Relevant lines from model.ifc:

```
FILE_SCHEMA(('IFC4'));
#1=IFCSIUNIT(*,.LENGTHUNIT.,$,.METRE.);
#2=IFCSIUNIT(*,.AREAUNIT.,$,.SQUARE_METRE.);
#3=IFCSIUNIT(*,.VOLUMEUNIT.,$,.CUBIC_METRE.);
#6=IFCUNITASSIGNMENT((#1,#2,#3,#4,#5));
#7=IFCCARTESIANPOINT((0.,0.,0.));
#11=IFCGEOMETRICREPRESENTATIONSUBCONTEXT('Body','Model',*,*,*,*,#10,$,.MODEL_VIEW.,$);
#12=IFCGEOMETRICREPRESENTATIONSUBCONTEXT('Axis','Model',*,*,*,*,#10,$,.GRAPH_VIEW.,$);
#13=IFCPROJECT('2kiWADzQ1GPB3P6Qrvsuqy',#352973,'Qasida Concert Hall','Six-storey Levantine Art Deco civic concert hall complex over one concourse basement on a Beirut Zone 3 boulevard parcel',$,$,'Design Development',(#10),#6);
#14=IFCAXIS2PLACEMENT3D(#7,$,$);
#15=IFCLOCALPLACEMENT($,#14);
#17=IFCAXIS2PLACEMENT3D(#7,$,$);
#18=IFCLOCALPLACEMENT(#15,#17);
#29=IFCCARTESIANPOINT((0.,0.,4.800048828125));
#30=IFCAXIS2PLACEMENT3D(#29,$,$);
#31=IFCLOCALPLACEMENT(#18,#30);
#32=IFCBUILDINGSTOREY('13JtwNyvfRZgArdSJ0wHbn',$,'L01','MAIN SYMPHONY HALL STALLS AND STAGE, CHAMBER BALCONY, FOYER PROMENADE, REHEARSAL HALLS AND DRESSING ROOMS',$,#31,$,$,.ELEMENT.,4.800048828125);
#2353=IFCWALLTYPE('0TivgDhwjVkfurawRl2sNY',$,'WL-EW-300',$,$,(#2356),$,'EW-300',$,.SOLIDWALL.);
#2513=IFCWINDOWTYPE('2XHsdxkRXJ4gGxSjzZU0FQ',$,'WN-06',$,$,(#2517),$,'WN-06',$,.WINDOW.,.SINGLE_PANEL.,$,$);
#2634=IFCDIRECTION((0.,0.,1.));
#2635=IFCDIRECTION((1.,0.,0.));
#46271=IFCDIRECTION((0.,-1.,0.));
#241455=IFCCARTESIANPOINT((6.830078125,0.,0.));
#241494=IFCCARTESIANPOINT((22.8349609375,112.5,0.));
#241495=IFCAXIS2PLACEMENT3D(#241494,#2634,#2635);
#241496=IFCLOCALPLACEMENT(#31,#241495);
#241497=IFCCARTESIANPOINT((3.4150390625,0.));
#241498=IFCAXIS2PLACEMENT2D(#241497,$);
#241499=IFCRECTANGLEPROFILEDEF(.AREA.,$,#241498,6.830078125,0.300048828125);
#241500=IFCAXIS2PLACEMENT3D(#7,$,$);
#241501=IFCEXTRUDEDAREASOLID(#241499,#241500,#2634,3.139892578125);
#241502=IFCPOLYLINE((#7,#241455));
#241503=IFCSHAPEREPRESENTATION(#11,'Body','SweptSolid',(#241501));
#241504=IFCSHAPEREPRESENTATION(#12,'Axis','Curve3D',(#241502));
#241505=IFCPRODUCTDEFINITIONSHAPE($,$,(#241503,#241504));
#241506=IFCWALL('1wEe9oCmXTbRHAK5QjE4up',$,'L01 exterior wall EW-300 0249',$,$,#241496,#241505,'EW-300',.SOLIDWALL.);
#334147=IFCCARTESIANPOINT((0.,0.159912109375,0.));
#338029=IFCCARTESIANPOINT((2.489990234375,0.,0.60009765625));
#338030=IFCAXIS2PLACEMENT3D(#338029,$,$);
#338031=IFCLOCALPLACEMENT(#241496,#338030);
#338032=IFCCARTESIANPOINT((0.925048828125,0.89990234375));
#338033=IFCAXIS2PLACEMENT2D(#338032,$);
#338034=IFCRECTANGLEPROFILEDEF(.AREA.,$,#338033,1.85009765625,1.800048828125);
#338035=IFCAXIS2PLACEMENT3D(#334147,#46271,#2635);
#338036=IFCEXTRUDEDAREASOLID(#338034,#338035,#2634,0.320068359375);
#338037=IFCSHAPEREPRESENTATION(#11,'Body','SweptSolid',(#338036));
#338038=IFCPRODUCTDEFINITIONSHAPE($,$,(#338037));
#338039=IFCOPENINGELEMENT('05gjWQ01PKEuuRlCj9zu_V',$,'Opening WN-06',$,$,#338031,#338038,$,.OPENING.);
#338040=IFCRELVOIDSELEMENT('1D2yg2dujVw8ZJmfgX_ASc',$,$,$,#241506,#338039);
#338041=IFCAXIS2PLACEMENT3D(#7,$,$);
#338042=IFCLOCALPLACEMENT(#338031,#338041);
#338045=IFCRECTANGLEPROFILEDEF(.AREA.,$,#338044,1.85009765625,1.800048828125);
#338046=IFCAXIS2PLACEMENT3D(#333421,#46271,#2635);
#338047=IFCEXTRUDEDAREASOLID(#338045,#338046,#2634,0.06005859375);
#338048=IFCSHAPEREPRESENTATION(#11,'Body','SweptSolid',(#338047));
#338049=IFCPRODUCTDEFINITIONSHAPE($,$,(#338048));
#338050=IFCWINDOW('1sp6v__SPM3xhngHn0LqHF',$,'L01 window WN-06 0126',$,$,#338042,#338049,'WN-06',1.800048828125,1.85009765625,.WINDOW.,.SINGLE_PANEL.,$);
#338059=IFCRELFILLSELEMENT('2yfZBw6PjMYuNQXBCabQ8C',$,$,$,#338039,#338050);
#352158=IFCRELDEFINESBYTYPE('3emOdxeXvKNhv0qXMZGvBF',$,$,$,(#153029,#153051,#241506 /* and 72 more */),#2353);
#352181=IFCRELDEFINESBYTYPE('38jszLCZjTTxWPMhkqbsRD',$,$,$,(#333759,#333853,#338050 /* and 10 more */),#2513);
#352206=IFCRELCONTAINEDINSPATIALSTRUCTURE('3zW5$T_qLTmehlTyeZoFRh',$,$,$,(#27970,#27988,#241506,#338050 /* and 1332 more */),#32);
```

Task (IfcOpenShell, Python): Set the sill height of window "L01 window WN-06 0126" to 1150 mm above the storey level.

```python
import numpy as np
import ifcopenshell
import ifcopenshell.api.geometry
import ifcopenshell.geom
import ifcopenshell.util.element
import ifcopenshell.util.placement
import ifcopenshell.util.shape
import ifcopenshell.util.unit

model = ifcopenshell.open("model.ifc")
unit_scale = ifcopenshell.util.unit.calculate_unit_scale(model)

window = model.by_guid("1sp6v__SPM3xhngHn0LqHF")
opening = window.FillsVoids[0].RelatingOpeningElement
storey = ifcopenshell.util.element.get_container(window, ifc_class="IfcBuildingStorey")
level = ifcopenshell.util.placement.get_local_placement(storey.ObjectPlacement)[2, 3]

# The opening's origin need not be at the sill, so measure its lowest point.
shape = ifcopenshell.geom.create_shape(ifcopenshell.geom.settings(), opening)
bottom = ifcopenshell.util.shape.get_shape_bottom_elevation(shape, shape.geometry) / unit_scale
dz = level + 1.15 / unit_scale - bottom

shift = np.array([0.0, 0.0, dz])
# The window is placed relative to its opening, so it follows when the opening moves.
matrix = ifcopenshell.util.placement.get_local_placement(opening.ObjectPlacement)
matrix[:3, 3] += shift
ifcopenshell.api.geometry.edit_object_placement(
    model, product=opening, matrix=matrix, is_si=False, should_transform_children=True
)

print(f"moved by {dz * unit_scale:+.3f} m")

model.write("model_edited.ifc")
```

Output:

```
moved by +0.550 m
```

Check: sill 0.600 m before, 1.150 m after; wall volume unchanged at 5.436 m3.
